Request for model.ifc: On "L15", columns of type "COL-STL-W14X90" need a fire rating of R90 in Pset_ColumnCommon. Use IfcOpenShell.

First a look at what the model holds.

```python
import ifcopenshell
import ifcopenshell.util.element

model = ifcopenshell.open("model.ifc")
print(model.schema)
storey = next(s for s in model.by_type("IfcBuildingStorey") if s.Name == "L15")
columns = [e for e in ifcopenshell.util.element.get_decomposition(storey) if e.is_a("IfcColumn")]
seen = {}
for e in columns:
    element_type = ifcopenshell.util.element.get_type(e)
    key = (element_type.Name if element_type != e and element_type else None, ifcopenshell.util.element.get_pset(e, "Pset_ColumnCommon", "FireRating"))
    seen[key] = seen.get(key, 0) + 1
for (name, value), count in sorted(seen.items(), key=str):
    print(count, "x", name, "|", value)
```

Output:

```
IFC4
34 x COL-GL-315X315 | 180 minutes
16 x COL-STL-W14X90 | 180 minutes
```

```python
import ifcopenshell
import ifcopenshell.api.pset
import ifcopenshell.util.element

model = ifcopenshell.open("model.ifc")

storey = next(s for s in model.by_type("IfcBuildingStorey") if s.Name == "L15")
columns = [e for e in ifcopenshell.util.element.get_decomposition(storey) if e.is_a("IfcColumn")]

count = 0
for e in columns:
    element_type = ifcopenshell.util.element.get_type(e)
    if element_type in (None, e) or element_type.Name != "COL-STL-W14X90":
        continue
    # add_pset returns the element's existing set when there is one.
    pset = ifcopenshell.api.pset.add_pset(model, product=e, name="Pset_ColumnCommon")
    ifcopenshell.api.pset.edit_pset(model, pset=pset, properties={"FireRating": "R90"})
    count += 1

print(count, "columns updated")

model.write("model-out.ifc")
```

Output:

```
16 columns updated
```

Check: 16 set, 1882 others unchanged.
